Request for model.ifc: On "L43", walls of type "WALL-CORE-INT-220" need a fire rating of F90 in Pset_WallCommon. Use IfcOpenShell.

First a look at what the model holds.

```python
import ifcopenshell
import ifcopenshell.util.element

model = ifcopenshell.open("model.ifc")
print(model.schema)
storey = next(s for s in model.by_type("IfcBuildingStorey") if s.Name == "L43")
walls = [e for e in ifcopenshell.util.element.get_decomposition(storey) if e.is_a("IfcWall")]
seen = {}
for e in walls:
    element_type = ifcopenshell.util.element.get_type(e)
    key = (element_type.Name if element_type != e and element_type else None, ifcopenshell.util.element.get_pset(e, "Pset_WallCommon", "FireRating"))
    seen[key] = seen.get(key, 0) + 1
for (name, value), count in sorted(seen.items(), key=str):
    print(count, "x", name, "|", value)
```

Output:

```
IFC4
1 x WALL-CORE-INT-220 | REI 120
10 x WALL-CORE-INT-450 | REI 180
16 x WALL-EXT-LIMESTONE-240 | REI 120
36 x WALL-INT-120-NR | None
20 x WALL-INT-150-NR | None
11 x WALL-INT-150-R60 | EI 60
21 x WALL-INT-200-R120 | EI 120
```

```python
import ifcopenshell
import ifcopenshell.api.pset
import ifcopenshell.util.element

model = ifcopenshell.open("model.ifc")

storey = next(s for s in model.by_type("IfcBuildingStorey") if s.Name == "L43")
walls = [e for e in ifcopenshell.util.element.get_decomposition(storey) if e.is_a("IfcWall")]

count = 0
for e in walls:
    element_type = ifcopenshell.util.element.get_type(e)
    if element_type in (None, e) or element_type.Name != "WALL-CORE-INT-220":
        continue
    # add_pset returns the element's existing set when there is one.
    pset = ifcopenshell.api.pset.add_pset(model, product=e, name="Pset_WallCommon")
    ifcopenshell.api.pset.edit_pset(model, pset=pset, properties={"FireRating": "F90"})
    count += 1

print(count, "walls updated")

model.write("model_edited.ifc")
```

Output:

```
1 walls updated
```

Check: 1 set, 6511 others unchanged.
